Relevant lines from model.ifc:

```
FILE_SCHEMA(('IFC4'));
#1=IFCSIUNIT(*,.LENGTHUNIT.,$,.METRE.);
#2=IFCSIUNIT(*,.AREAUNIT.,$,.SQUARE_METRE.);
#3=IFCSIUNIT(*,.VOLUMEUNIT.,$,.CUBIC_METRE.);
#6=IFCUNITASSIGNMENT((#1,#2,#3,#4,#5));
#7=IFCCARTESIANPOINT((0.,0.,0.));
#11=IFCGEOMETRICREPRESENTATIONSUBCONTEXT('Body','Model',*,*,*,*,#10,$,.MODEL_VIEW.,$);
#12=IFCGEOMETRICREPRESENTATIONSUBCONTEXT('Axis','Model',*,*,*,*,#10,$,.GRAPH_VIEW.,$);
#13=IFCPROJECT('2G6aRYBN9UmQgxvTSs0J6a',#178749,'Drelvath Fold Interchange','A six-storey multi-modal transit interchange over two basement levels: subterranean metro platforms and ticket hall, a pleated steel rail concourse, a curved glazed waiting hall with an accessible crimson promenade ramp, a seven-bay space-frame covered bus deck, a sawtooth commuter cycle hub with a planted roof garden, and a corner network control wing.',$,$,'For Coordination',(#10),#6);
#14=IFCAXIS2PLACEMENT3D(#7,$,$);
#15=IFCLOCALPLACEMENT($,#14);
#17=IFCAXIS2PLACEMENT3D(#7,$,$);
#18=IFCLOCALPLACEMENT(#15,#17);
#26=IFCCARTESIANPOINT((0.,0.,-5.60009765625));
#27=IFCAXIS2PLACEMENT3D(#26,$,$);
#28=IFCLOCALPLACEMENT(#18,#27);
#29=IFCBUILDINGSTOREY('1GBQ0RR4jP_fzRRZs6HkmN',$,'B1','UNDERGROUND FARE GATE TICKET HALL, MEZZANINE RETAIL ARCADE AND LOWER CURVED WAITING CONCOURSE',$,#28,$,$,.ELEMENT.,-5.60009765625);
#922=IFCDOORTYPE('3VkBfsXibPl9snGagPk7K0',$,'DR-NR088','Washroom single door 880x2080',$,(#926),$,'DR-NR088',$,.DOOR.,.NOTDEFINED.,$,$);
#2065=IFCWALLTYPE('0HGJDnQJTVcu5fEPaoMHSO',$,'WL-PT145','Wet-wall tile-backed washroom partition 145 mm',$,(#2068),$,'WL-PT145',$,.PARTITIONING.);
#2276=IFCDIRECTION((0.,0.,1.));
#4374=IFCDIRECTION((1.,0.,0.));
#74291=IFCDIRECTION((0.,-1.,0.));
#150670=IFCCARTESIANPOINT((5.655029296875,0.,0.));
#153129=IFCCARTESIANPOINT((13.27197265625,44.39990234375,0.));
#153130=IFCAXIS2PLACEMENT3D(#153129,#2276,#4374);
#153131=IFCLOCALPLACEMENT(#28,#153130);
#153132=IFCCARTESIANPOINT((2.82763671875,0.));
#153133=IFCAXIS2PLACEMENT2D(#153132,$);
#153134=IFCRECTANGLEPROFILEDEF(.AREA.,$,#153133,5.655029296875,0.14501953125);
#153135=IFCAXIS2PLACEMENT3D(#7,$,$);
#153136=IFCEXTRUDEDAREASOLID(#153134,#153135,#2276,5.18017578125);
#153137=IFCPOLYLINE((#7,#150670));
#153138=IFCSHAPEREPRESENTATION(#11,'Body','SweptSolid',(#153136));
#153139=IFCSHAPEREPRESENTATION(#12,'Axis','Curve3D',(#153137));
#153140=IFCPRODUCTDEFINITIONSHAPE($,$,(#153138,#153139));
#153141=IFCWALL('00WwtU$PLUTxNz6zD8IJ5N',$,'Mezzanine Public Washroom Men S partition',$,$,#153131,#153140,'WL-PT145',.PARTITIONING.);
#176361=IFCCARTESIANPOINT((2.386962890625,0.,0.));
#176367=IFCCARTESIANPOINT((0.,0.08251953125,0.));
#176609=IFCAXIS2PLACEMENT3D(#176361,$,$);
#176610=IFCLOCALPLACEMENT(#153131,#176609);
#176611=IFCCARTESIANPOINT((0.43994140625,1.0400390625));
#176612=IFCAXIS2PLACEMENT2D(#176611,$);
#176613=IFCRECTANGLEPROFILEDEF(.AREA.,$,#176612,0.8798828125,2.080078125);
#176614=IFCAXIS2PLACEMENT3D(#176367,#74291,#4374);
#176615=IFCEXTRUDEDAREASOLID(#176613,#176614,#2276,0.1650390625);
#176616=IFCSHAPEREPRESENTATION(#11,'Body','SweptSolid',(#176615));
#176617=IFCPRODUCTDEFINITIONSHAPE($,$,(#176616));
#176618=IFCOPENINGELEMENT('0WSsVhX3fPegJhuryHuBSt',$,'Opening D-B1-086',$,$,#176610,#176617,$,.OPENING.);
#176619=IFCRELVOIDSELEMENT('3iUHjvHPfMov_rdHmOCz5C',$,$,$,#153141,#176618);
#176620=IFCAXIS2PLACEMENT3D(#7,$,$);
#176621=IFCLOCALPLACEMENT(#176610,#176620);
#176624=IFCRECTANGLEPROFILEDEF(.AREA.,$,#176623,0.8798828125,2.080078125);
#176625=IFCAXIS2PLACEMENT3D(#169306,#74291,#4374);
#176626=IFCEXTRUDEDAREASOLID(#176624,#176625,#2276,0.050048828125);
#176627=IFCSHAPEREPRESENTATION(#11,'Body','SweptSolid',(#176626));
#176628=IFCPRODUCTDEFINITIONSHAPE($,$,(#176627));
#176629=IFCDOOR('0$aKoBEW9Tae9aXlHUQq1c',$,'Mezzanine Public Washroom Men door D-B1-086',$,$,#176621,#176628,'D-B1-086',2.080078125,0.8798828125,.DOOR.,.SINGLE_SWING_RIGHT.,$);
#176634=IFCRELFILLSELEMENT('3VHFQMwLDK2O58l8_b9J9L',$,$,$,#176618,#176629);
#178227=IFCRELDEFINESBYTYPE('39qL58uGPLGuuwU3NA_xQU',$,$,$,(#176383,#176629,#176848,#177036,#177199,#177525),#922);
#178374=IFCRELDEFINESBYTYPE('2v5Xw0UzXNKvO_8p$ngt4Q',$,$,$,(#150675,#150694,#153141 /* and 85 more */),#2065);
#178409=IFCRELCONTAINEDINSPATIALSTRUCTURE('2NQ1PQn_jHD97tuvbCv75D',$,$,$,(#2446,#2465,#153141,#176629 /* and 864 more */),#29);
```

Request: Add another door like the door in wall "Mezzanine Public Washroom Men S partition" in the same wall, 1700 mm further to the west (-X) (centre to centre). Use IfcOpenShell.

```python
import ifcopenshell
import ifcopenshell.api.feature
import ifcopenshell.api.geometry
import ifcopenshell.api.root
import ifcopenshell.geom
import ifcopenshell.util.element
import ifcopenshell.util.placement
import ifcopenshell.util.shape
import ifcopenshell.util.unit

model = ifcopenshell.open("model.ifc")
unit_scale = ifcopenshell.util.unit.calculate_unit_scale(model)
settings = ifcopenshell.geom.settings()


def volume(element):
    """Net volume in cubic metres, openings subtracted."""
    shape = ifcopenshell.geom.create_shape(settings, element)
    return ifcopenshell.util.shape.get_volume(shape.geometry)


door = model.by_guid("0$aKoBEW9Tae9aXlHUQq1c")
opening = door.FillsVoids[0].RelatingOpeningElement
wall = opening.VoidsElements[0].RelatingBuildingElement
before = volume(wall)
shift = ifcopenshell.util.placement.get_local_placement(wall.ObjectPlacement)[:3, 0] * -1.7 / unit_scale

# copy_class copies the void relationship, type, container and properties, but no geometry.
new_opening = ifcopenshell.api.root.copy_class(model, product=opening)
new_opening.Representation = ifcopenshell.util.element.copy_deep(
    model, opening.Representation, exclude=["IfcGeometricRepresentationContext", "IfcRepresentationMap"]
)
new_door = ifcopenshell.api.root.copy_class(model, product=door)
new_door.Representation = ifcopenshell.util.element.copy_deep(
    model, door.Representation, exclude=["IfcGeometricRepresentationContext", "IfcRepresentationMap"]
)
new_door.Tag = None
ifcopenshell.api.feature.add_filling(model, opening=new_opening, element=new_door)

for old, new in ((opening, new_opening), (door, new_door)):
    matrix = ifcopenshell.util.placement.get_local_placement(old.ObjectPlacement)
    matrix[:3, 3] += shift
    ifcopenshell.api.geometry.edit_object_placement(model, product=new, matrix=matrix, is_si=False)

after = volume(wall)

print(f"wall volume {before:.3f} -> {after:.3f} m3")

model.write("model_rev.ifc")
```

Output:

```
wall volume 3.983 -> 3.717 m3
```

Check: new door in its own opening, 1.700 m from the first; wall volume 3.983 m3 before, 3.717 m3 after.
